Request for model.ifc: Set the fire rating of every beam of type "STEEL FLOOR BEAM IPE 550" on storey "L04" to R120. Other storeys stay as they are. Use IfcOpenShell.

First a look at what the model holds.

```python
import ifcopenshell
import ifcopenshell.util.element

model = ifcopenshell.open("model.ifc")
print(model.schema)
storey = next(s for s in model.by_type("IfcBuildingStorey") if s.Name == "L04")
beams = [e for e in ifcopenshell.util.element.get_decomposition(storey) if e.is_a("IfcBeam")]
seen = {}
for e in beams:
    element_type = ifcopenshell.util.element.get_type(e)
    key = (element_type.Name if element_type != e and element_type else None, ifcopenshell.util.element.get_pset(e, "Pset_BeamCommon", "FireRating"))
    seen[key] = seen.get(key, 0) + 1
for (name, value), count in sorted(seen.items(), key=str):
    print(count, "x", name, "|", value)
```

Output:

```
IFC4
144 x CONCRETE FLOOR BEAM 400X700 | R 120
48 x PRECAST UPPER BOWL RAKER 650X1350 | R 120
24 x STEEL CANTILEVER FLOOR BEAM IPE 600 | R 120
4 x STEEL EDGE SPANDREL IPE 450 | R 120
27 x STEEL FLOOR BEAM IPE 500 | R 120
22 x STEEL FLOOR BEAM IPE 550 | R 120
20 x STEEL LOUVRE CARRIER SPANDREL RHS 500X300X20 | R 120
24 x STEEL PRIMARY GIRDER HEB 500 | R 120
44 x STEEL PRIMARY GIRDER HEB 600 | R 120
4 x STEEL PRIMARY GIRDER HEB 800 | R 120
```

```python
import ifcopenshell
import ifcopenshell.api.pset
import ifcopenshell.util.element

model = ifcopenshell.open("model.ifc")

storey = next(s for s in model.by_type("IfcBuildingStorey") if s.Name == "L04")
beams = [e for e in ifcopenshell.util.element.get_decomposition(storey) if e.is_a("IfcBeam")]

count = 0
for e in beams:
    element_type = ifcopenshell.util.element.get_type(e)
    if element_type in (None, e) or element_type.Name != "STEEL FLOOR BEAM IPE 550":
        continue
    # add_pset returns the element's existing set when there is one.
    pset = ifcopenshell.api.pset.add_pset(model, product=e, name="Pset_BeamCommon")
    ifcopenshell.api.pset.edit_pset(model, pset=pset, properties={"FireRating": "R120"})
    count += 1

print(count, "beams updated")

model.write("model_edited.ifc")
```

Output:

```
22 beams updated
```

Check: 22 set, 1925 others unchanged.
